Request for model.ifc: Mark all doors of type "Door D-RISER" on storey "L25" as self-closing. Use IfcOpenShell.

First a look at what the model holds.

```python
import ifcopenshell
import ifcopenshell.util.element

model = ifcopenshell.open("model.ifc")
print(model.schema)
storey = next(s for s in model.by_type("IfcBuildingStorey") if s.Name == "L25")
doors = [e for e in ifcopenshell.util.element.get_decomposition(storey) if e.is_a("IfcDoor")]
seen = {}
for e in doors:
    element_type = ifcopenshell.util.element.get_type(e)
    key = (element_type.Name if element_type != e and element_type else None, ifcopenshell.util.element.get_pset(e, "Pset_DoorCommon", "SelfClosing"))
    seen[key] = seen.get(key, 0) + 1
for (name, value), count in sorted(seen.items(), key=str):
    print(count, "x", name, "|", value)
```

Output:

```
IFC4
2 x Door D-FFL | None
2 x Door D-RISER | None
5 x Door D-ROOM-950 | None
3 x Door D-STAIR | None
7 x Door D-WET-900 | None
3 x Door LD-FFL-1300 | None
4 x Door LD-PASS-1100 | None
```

```python
import ifcopenshell
import ifcopenshell.api.pset
import ifcopenshell.util.element

model = ifcopenshell.open("model.ifc")

storey = next(s for s in model.by_type("IfcBuildingStorey") if s.Name == "L25")
doors = [e for e in ifcopenshell.util.element.get_decomposition(storey) if e.is_a("IfcDoor")]

count = 0
for e in doors:
    element_type = ifcopenshell.util.element.get_type(e)
    if element_type in (None, e) or element_type.Name != "Door D-RISER":
        continue
    found = ifcopenshell.util.element.get_pset(e, "Pset_DoorCommon", should_inherit=False)
    if found:
        pset = model.by_id(found["id"])
        if len(ifcopenshell.util.element.get_elements_by_pset(pset)) > 1:
            pset = ifcopenshell.api.pset.unshare_pset(model, products=[e], pset=pset)[0]
    else:
        pset = ifcopenshell.api.pset.add_pset(model, product=e, name="Pset_DoorCommon")
    ifcopenshell.api.pset.edit_pset(model, pset=pset, properties={"SelfClosing": True})
    count += 1

print(count, "doors updated")

model.write("model_edited.ifc")
```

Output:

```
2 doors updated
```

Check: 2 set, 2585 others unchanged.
